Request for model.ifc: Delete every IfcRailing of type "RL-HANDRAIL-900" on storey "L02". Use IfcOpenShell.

First a look at what the model holds.

```python
import ifcopenshell
import ifcopenshell.util.element

model = ifcopenshell.open("model.ifc")
print(model.schema)
storey = next(s for s in model.by_type("IfcBuildingStorey") if s.Name == "L02")
railings = [e for e in ifcopenshell.util.element.get_decomposition(storey) if e.is_a("IfcRailing")]
seen = {}
for e in railings:
    element_type = ifcopenshell.util.element.get_type(e)
    name = element_type.Name if element_type not in (None, e) else None
    seen[name] = seen.get(name, 0) + 1
for name, count in sorted(seen.items(), key=str):
    print(count, "x", name)
```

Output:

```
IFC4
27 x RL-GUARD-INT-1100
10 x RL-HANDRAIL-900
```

```python
import ifcopenshell
import ifcopenshell.api.root
import ifcopenshell.util.element

model = ifcopenshell.open("model.ifc")

storey = next(s for s in model.by_type("IfcBuildingStorey") if s.Name == "L02")
railings = [e for e in ifcopenshell.util.element.get_decomposition(storey) if e.is_a("IfcRailing")]
targets = [e for e in railings if (t := ifcopenshell.util.element.get_type(e)) not in (None, e) and t.Name == "RL-HANDRAIL-900"]

for e in targets:
    ifcopenshell.api.root.remove_product(model, product=e)
print(len(targets), "removed")

model.write("model_edited.ifc")
```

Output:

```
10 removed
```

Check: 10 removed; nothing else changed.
